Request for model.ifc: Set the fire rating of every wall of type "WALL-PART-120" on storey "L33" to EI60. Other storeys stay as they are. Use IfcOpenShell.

First a look at what the model holds.

```python
import ifcopenshell
import ifcopenshell.util.element

model = ifcopenshell.open("model.ifc")
print(model.schema)
storey = next(s for s in model.by_type("IfcBuildingStorey") if s.Name == "L33")
walls = [e for e in ifcopenshell.util.element.get_decomposition(storey) if e.is_a("IfcWall")]
seen = {}
for e in walls:
    element_type = ifcopenshell.util.element.get_type(e)
    key = (element_type.Name if element_type != e and element_type else None, ifcopenshell.util.element.get_pset(e, "Pset_WallCommon", "FireRating"))
    seen[key] = seen.get(key, 0) + 1
for (name, value), count in sorted(seen.items(), key=str):
    print(count, "x", name, "|", value)
```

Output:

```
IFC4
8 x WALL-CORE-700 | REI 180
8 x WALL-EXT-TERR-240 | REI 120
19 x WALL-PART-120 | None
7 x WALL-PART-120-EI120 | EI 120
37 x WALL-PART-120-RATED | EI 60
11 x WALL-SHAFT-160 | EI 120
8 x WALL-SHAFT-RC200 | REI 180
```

```python
import ifcopenshell
import ifcopenshell.api.pset
import ifcopenshell.util.element

model = ifcopenshell.open("model.ifc")

storey = next(s for s in model.by_type("IfcBuildingStorey") if s.Name == "L33")
walls = [e for e in ifcopenshell.util.element.get_decomposition(storey) if e.is_a("IfcWall")]

count = 0
for e in walls:
    element_type = ifcopenshell.util.element.get_type(e)
    if element_type in (None, e) or element_type.Name != "WALL-PART-120":
        continue
    # add_pset returns the element's existing set when there is one.
    pset = ifcopenshell.api.pset.add_pset(model, product=e, name="Pset_WallCommon")
    ifcopenshell.api.pset.edit_pset(model, pset=pset, properties={"FireRating": "EI60"})
    count += 1

print(count, "walls updated")

model.write("model_v2.ifc")
```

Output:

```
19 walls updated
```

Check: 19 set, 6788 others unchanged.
